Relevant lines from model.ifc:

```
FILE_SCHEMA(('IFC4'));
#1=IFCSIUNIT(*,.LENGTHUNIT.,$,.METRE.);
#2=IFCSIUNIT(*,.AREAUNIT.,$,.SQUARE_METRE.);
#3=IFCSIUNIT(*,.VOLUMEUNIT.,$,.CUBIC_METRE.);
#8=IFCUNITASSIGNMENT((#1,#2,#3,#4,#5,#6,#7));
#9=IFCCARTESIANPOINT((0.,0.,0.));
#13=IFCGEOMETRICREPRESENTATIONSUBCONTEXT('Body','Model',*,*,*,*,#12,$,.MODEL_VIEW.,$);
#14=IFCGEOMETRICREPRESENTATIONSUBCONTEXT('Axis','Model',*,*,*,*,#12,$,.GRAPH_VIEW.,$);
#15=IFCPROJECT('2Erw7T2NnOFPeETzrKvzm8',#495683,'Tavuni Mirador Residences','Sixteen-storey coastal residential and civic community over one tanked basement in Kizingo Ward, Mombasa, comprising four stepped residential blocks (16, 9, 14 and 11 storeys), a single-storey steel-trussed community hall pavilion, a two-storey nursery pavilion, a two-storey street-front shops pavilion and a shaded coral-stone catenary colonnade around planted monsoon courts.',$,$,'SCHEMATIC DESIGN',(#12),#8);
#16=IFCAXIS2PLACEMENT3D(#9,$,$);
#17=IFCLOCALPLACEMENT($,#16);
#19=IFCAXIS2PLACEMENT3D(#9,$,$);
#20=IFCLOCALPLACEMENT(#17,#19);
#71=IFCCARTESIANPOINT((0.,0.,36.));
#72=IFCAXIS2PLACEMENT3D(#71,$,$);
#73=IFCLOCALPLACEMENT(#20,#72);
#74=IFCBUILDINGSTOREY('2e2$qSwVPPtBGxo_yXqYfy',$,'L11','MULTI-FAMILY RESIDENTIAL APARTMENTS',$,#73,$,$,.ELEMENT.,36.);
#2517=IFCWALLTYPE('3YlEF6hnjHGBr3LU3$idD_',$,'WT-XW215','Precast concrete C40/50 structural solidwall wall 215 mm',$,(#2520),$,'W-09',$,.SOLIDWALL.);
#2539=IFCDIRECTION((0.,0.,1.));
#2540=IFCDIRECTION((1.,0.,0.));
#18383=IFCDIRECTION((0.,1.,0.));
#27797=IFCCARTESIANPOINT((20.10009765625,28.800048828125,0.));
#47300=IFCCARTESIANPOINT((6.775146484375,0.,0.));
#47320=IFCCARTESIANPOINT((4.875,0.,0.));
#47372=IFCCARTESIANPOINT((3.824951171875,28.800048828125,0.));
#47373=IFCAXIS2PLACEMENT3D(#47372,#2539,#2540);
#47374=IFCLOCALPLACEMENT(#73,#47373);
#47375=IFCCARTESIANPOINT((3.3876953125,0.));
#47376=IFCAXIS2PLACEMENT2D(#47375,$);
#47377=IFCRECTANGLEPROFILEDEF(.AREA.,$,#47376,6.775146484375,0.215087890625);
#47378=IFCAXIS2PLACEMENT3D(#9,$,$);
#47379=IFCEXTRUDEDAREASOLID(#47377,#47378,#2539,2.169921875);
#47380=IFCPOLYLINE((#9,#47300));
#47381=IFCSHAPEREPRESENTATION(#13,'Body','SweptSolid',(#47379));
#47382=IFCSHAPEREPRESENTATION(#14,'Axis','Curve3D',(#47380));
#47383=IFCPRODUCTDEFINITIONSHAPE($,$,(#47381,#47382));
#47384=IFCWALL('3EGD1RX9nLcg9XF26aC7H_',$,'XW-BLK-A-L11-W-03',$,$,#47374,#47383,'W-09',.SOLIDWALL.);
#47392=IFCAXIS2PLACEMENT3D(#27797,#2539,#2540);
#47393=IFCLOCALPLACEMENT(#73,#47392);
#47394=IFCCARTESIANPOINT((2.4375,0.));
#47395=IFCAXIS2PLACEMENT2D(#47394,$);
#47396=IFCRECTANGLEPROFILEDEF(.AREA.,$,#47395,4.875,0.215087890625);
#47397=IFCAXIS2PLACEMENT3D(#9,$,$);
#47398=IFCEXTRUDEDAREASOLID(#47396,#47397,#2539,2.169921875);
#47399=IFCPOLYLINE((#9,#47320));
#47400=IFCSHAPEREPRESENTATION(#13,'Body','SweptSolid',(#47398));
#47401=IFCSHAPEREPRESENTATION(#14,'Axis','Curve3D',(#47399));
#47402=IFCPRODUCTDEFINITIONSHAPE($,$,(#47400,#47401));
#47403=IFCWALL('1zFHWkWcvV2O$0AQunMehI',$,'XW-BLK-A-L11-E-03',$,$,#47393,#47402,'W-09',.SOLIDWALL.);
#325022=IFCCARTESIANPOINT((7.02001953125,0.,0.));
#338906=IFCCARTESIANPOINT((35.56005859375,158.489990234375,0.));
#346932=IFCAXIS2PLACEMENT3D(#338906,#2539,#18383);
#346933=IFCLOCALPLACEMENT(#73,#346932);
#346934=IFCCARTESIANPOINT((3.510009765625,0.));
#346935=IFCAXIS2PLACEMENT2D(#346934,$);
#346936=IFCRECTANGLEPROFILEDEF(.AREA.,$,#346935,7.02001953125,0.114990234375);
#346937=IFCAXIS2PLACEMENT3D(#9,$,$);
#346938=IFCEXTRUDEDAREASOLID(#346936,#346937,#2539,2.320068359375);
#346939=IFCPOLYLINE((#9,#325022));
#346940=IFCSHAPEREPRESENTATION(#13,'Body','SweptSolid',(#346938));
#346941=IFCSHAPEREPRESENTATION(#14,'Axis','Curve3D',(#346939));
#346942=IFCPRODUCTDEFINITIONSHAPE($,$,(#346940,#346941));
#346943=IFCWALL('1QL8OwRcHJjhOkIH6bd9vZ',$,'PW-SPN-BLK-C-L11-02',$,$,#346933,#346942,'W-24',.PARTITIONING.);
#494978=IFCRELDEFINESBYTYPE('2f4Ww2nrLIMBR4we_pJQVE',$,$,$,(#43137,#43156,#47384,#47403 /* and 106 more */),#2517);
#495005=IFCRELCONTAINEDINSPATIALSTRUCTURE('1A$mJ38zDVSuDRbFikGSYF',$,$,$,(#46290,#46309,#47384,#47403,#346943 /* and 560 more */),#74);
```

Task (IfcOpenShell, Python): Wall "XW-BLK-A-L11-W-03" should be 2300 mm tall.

```python
import ifcopenshell
import ifcopenshell.geom
import ifcopenshell.util.representation
import ifcopenshell.util.shape

model = ifcopenshell.open("model.ifc")
settings = ifcopenshell.geom.settings()


def volume(element):
    """Net volume in cubic metres, openings subtracted."""
    shape = ifcopenshell.geom.create_shape(settings, element)
    return ifcopenshell.util.shape.get_volume(shape.geometry)


wall = model.by_id(47384)
before = volume(wall)

body = ifcopenshell.util.representation.get_representation(wall, "Model", "Body")
solid = body.Items[0]
old_height = solid.Depth
solid.Depth = 2.3
after = volume(wall)

print(f"height {old_height:g} -> {solid.Depth:g}, volume {before:.3f} -> {after:.3f} m3")

model.write("model_v2.ifc")
```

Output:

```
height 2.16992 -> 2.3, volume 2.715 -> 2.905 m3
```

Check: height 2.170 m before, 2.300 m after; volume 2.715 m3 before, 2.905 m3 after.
